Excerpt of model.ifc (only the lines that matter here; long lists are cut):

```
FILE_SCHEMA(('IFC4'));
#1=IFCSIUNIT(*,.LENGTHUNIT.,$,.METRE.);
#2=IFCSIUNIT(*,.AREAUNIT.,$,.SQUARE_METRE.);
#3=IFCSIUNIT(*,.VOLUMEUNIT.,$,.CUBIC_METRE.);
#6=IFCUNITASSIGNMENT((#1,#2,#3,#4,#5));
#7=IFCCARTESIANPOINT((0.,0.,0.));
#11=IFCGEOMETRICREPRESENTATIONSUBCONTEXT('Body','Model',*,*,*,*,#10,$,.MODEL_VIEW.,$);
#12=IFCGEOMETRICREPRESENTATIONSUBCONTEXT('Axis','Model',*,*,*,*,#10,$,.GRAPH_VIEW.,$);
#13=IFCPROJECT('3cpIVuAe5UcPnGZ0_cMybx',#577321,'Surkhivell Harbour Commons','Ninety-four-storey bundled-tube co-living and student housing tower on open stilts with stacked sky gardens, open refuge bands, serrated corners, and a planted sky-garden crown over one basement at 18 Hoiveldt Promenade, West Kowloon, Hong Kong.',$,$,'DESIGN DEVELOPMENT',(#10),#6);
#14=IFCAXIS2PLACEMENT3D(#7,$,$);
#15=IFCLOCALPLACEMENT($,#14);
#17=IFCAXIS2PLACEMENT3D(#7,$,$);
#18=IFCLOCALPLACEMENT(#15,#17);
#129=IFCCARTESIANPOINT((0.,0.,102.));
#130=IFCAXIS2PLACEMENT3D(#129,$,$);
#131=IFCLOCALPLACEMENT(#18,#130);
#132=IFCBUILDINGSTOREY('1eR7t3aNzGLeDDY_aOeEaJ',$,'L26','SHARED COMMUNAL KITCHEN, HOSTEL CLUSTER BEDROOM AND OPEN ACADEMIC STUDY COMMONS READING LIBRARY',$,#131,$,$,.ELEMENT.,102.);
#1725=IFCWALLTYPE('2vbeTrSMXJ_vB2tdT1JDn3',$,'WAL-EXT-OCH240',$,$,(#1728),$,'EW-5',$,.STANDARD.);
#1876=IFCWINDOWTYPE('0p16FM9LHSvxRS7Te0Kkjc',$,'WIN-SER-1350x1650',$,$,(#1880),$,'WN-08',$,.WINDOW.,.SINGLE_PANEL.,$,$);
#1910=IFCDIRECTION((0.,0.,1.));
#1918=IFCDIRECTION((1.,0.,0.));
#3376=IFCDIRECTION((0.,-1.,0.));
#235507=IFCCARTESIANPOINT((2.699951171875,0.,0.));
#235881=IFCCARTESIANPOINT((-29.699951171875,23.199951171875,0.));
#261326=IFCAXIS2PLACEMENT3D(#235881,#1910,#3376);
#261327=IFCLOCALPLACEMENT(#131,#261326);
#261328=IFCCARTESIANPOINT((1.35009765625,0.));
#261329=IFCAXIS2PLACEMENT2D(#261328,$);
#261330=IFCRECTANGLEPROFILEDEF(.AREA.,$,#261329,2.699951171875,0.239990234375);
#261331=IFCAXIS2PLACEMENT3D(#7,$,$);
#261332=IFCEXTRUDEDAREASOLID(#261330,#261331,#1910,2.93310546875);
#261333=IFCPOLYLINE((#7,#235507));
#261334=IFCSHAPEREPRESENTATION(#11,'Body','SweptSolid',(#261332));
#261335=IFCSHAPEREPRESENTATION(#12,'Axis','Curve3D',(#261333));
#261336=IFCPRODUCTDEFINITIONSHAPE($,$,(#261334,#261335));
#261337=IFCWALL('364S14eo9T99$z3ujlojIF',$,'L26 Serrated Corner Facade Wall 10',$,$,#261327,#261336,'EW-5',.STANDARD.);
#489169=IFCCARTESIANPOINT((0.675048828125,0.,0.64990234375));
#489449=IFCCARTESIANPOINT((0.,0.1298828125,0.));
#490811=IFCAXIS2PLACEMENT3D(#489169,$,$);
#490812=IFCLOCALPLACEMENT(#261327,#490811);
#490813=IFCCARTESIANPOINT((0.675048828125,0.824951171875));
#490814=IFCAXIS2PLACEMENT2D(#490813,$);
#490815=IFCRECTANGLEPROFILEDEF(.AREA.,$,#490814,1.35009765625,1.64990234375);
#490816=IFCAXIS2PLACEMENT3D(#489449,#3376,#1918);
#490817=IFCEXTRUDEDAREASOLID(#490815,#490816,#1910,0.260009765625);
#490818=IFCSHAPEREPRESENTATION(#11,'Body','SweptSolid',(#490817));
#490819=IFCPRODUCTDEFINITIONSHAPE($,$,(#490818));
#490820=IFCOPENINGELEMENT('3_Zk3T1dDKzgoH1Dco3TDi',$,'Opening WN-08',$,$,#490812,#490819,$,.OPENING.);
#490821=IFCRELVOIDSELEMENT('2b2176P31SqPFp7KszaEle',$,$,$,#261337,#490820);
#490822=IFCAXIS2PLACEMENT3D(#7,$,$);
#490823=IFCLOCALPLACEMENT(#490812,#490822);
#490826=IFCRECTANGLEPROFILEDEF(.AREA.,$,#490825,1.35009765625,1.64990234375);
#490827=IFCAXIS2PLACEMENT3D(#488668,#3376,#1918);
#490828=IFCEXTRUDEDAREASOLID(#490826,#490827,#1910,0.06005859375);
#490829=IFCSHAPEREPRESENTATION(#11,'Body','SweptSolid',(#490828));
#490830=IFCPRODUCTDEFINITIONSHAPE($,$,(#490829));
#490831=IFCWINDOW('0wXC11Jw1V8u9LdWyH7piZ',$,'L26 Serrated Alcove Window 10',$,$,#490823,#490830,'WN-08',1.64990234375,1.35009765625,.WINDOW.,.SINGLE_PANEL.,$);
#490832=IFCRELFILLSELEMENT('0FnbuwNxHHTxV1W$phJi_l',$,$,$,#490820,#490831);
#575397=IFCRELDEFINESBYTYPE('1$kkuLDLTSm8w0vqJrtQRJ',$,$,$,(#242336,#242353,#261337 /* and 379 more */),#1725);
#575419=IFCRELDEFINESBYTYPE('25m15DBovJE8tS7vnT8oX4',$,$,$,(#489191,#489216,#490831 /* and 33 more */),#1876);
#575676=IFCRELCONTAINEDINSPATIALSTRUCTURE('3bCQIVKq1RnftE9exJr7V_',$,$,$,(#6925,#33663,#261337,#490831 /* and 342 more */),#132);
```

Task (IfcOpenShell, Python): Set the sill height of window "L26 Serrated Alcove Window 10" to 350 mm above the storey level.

```python
import numpy as np
import ifcopenshell
import ifcopenshell.api.geometry
import ifcopenshell.geom
import ifcopenshell.util.element
import ifcopenshell.util.placement
import ifcopenshell.util.shape
import ifcopenshell.util.unit

model = ifcopenshell.open("model.ifc")
unit_scale = ifcopenshell.util.unit.calculate_unit_scale(model)

window = model.by_guid("0wXC11Jw1V8u9LdWyH7piZ")
opening = window.FillsVoids[0].RelatingOpeningElement
storey = ifcopenshell.util.element.get_container(window, ifc_class="IfcBuildingStorey")
level = ifcopenshell.util.placement.get_local_placement(storey.ObjectPlacement)[2, 3]

# The opening's origin need not be at the sill, so measure its lowest point.
shape = ifcopenshell.geom.create_shape(ifcopenshell.geom.settings(), opening)
bottom = ifcopenshell.util.shape.get_shape_bottom_elevation(shape, shape.geometry) / unit_scale
dz = level + 0.35 / unit_scale - bottom

shift = np.array([0.0, 0.0, dz])
# The window is placed relative to its opening, so it follows when the opening moves.
matrix = ifcopenshell.util.placement.get_local_placement(opening.ObjectPlacement)
matrix[:3, 3] += shift
ifcopenshell.api.geometry.edit_object_placement(
    model, product=opening, matrix=matrix, is_si=False, should_transform_children=True
)

print(f"moved by {dz * unit_scale:+.3f} m")

model.write("model_updated.ifc")
```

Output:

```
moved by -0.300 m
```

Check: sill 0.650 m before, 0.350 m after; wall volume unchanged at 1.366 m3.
